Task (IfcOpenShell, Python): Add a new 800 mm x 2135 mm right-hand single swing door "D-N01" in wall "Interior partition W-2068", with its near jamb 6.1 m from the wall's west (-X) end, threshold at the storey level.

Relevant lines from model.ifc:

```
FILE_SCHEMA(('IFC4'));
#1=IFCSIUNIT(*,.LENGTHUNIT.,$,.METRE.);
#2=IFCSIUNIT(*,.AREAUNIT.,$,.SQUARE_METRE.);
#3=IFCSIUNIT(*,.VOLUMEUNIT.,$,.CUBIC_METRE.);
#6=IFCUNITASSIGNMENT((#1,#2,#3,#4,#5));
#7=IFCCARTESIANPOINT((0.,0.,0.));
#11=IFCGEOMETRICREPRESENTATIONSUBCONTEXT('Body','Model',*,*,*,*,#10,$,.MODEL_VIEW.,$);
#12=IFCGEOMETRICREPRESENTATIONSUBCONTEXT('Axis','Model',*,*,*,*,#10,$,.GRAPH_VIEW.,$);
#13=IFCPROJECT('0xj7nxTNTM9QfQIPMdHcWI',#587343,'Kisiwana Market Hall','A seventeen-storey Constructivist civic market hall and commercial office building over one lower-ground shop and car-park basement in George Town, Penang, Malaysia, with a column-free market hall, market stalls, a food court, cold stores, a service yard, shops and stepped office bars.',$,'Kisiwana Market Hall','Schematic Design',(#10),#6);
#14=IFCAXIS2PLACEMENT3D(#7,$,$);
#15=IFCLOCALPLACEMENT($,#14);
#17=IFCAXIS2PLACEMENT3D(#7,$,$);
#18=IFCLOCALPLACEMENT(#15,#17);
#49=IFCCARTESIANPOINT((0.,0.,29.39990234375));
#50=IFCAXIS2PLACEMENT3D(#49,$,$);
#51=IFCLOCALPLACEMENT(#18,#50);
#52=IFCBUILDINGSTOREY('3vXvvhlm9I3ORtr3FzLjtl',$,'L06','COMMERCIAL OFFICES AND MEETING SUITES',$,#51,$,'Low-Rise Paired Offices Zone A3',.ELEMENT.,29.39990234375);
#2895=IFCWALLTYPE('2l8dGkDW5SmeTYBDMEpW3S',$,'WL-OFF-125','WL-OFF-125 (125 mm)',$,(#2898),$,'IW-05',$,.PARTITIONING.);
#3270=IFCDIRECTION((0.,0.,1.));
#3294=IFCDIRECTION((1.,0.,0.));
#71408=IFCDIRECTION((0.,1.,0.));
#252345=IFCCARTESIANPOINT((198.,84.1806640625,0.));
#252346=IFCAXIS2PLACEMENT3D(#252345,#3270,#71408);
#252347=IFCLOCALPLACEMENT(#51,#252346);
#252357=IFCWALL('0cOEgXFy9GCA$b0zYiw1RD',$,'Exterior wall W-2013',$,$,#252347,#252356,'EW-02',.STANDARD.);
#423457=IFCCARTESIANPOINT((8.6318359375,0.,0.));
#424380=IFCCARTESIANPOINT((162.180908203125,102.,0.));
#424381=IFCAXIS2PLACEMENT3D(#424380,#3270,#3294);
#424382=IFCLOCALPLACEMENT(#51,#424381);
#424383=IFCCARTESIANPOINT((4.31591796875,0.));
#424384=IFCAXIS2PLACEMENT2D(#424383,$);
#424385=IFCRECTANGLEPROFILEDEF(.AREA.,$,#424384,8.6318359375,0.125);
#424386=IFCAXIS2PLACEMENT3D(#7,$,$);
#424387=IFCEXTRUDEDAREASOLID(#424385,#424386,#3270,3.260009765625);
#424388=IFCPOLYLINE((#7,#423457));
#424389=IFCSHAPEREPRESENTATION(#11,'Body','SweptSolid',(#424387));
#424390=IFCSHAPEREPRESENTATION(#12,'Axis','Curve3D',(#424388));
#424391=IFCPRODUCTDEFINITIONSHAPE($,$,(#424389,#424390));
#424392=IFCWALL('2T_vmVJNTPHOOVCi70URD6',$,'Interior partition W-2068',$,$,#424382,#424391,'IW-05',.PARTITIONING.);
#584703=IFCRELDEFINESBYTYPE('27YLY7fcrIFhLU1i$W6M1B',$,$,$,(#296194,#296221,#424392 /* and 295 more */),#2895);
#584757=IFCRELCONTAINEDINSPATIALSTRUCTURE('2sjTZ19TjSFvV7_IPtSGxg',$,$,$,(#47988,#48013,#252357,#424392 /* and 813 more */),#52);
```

```python
import numpy as np
import ifcopenshell
import ifcopenshell.api.feature
import ifcopenshell.api.geometry
import ifcopenshell.api.root
import ifcopenshell.api.spatial
import ifcopenshell.geom
import ifcopenshell.util.element
import ifcopenshell.util.placement
import ifcopenshell.util.representation
import ifcopenshell.util.shape
import ifcopenshell.util.unit

model = ifcopenshell.open("model.ifc")
unit_scale = ifcopenshell.util.unit.calculate_unit_scale(model)
settings = ifcopenshell.geom.settings()


def volume(element):
    """Net volume in cubic metres, openings subtracted."""
    shape = ifcopenshell.geom.create_shape(settings, element)
    return ifcopenshell.util.shape.get_volume(shape.geometry)


wall = model.by_guid("2T_vmVJNTPHOOVCi70URD6")
storey = ifcopenshell.util.element.get_container(wall, ifc_class="IfcBuildingStorey")
context = ifcopenshell.util.representation.get_context(model, "Model", "Body", "MODEL_VIEW")
before = volume(wall)

width, height, from_end, sill = 0.8, 2.135, 6.1, 0.0  # metres

# The wall runs along its own X axis, and the end named is its -X end.
wall_shape = ifcopenshell.geom.create_shape(settings, wall)
x, y, z = ifcopenshell.util.shape.get_vertices(wall_shape.geometry).T
start = x.min() + from_end
face, thickness = float(y.min()), float(y.max() - y.min())
wall_matrix = ifcopenshell.util.placement.get_local_placement(wall.ObjectPlacement)
level = ifcopenshell.util.placement.get_local_placement(storey.ObjectPlacement)[2, 3]


def in_wall(x, y):
    """Placement at x, y metres in the wall's axes, at sill height."""
    matrix = wall_matrix.copy()
    matrix[:, 3] = wall_matrix @ np.array([x / unit_scale, y / unit_scale, 0.0, 1.0])
    matrix[2, 3] = level + sill / unit_scale
    return matrix


# Opening: a box that overshoots both wall faces by 50 mm.
opening = ifcopenshell.api.root.create_entity(model, ifc_class="IfcOpeningElement", predefined_type="OPENING")
box = ifcopenshell.api.geometry.add_wall_representation(
    model, context=context, length=width, height=height, thickness=thickness + 0.1
)
ifcopenshell.api.geometry.assign_representation(model, product=opening, representation=box)
ifcopenshell.api.geometry.edit_object_placement(model, product=opening, matrix=in_wall(start, face - 0.05), is_si=False)
ifcopenshell.api.feature.add_feature(model, feature=opening, element=wall)

door = ifcopenshell.api.root.create_entity(model, ifc_class="IfcDoor", name="D-N01", predefined_type="DOOR")
door.OverallWidth, door.OverallHeight = width / unit_scale, height / unit_scale
door.OperationType = "SINGLE_SWING_RIGHT"
body = ifcopenshell.api.geometry.add_door_representation(
    model,
    context=context,
    overall_width=door.OverallWidth,
    overall_height=door.OverallHeight,
    operation_type="SINGLE_SWING_RIGHT",
    lining_properties={"LiningDepth": thickness / unit_scale, "ThresholdDepth": thickness / unit_scale},
)
ifcopenshell.api.geometry.assign_representation(model, product=door, representation=body)
ifcopenshell.api.spatial.assign_container(model, products=[door], relating_structure=storey)
ifcopenshell.api.feature.add_filling(model, opening=opening, element=door)

# The lining spans the wall, so the door starts at the wall face.
ifcopenshell.api.geometry.edit_object_placement(model, product=door, matrix=in_wall(start, face), is_si=False)

after = volume(wall)

print(f"wall volume {before:.3f} -> {after:.3f} m3")

model.write("model-out.ifc")
```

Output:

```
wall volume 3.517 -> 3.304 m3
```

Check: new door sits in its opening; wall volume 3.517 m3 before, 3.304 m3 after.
